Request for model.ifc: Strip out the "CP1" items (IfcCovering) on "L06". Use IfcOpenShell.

First a look at what the model holds.

```python
import ifcopenshell
import ifcopenshell.util.element

model = ifcopenshell.open("model.ifc")
print(model.schema)
storey = next(s for s in model.by_type("IfcBuildingStorey") if s.Name == "L06")
coverings = [e for e in ifcopenshell.util.element.get_decomposition(storey) if e.is_a("IfcCovering")]
seen = {}
for e in coverings:
    element_type = ifcopenshell.util.element.get_type(e)
    name = element_type.Name if element_type not in (None, e) else None
    seen[name] = seen.get(name, 0) + 1
for name, count in sorted(seen.items(), key=str):
    print(count, "x", name)
```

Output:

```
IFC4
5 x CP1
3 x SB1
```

```python
import ifcopenshell
import ifcopenshell.api.root
import ifcopenshell.util.element

model = ifcopenshell.open("model.ifc")

storey = next(s for s in model.by_type("IfcBuildingStorey") if s.Name == "L06")
coverings = [e for e in ifcopenshell.util.element.get_decomposition(storey) if e.is_a("IfcCovering")]
targets = [e for e in coverings if (t := ifcopenshell.util.element.get_type(e)) not in (None, e) and t.Name == "CP1"]

for e in targets:
    ifcopenshell.api.root.remove_product(model, product=e)
print(len(targets), "removed")

model.write("model_rev.ifc")
```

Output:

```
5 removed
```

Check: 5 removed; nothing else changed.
